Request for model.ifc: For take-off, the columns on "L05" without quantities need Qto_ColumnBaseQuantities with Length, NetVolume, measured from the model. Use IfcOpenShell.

First a look at what the model holds.

```python
import ifcopenshell
import ifcopenshell.util.element
import ifcopenshell.util.unit

model = ifcopenshell.open("model.ifc")
print(model.schema)
for unit_type in ("LENGTHUNIT", "AREAUNIT", "VOLUMEUNIT"):
    print(unit_type, ifcopenshell.util.unit.calculate_unit_scale(model, unit_type))
storey = next(s for s in model.by_type("IfcBuildingStorey") if s.Name == "L05")
columns = [e for e in ifcopenshell.util.element.get_decomposition(storey) if e.is_a("IfcColumn")]
for e in sorted(columns, key=lambda e: e.id()):
    print(e.id(), e.is_a(), e.Name, list(ifcopenshell.util.element.get_psets(e, qtos_only=True)), sep=" | ")
```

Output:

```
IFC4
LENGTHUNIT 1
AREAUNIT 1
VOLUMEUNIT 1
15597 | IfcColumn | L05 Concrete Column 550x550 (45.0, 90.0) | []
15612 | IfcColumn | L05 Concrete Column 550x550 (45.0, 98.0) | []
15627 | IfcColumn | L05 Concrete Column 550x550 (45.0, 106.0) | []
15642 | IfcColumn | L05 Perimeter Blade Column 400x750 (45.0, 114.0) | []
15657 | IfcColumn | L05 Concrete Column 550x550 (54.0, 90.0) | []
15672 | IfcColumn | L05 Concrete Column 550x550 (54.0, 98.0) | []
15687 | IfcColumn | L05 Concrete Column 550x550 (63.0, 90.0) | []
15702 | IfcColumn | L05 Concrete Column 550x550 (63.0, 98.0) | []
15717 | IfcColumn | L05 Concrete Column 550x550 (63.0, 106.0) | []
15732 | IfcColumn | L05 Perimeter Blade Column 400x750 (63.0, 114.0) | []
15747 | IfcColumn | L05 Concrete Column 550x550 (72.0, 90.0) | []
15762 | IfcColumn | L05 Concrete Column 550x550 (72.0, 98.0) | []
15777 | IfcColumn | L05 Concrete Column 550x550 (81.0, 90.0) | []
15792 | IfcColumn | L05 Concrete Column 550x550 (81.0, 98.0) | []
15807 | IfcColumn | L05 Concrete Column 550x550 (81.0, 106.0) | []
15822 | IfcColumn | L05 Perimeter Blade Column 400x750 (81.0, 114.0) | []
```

```python
import ifcopenshell
import ifcopenshell.api.pset
import ifcopenshell.geom
import ifcopenshell.util.element
import ifcopenshell.util.shape
import ifcopenshell.util.unit

model = ifcopenshell.open("model.ifc")
unit_scale = ifcopenshell.util.unit.calculate_unit_scale(model)
volume_scale = ifcopenshell.util.unit.calculate_unit_scale(model, "VOLUMEUNIT")
settings = ifcopenshell.geom.settings()

storey = next(s for s in model.by_type("IfcBuildingStorey") if s.Name == "L05")
columns = [e for e in ifcopenshell.util.element.get_decomposition(storey) if e.is_a("IfcColumn")]

for e in sorted(columns, key=lambda e: e.id()):
    if ifcopenshell.util.element.get_psets(e, qtos_only=True, should_inherit=False):
        continue
    # Geometry comes back in metres, in the element's own axes.
    shape = ifcopenshell.geom.create_shape(settings, e)
    values = {
        "Length": ifcopenshell.util.shape.get_z(shape.geometry) / unit_scale,
        "NetVolume": ifcopenshell.util.shape.get_volume(shape.geometry) / volume_scale,
    }
    qto = ifcopenshell.api.pset.add_qto(model, product=e, name="Qto_ColumnBaseQuantities")
    ifcopenshell.api.pset.edit_qto(model, qto=qto, properties=values)
    print(e.id(), {k: round(v, 3) for k, v in values.items()})

model.write("model_v2.ifc")
```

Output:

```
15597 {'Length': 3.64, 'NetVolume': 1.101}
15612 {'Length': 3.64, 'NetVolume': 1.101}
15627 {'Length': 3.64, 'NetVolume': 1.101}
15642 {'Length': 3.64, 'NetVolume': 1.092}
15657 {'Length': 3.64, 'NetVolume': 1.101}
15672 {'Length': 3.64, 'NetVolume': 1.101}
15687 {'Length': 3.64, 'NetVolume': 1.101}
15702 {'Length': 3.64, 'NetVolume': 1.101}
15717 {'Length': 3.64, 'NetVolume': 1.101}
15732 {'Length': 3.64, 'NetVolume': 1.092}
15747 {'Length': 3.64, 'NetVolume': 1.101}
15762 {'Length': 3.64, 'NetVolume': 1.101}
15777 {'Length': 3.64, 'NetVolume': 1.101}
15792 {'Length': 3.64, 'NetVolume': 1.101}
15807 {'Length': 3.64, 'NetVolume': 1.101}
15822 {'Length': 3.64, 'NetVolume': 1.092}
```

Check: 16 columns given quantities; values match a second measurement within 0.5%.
